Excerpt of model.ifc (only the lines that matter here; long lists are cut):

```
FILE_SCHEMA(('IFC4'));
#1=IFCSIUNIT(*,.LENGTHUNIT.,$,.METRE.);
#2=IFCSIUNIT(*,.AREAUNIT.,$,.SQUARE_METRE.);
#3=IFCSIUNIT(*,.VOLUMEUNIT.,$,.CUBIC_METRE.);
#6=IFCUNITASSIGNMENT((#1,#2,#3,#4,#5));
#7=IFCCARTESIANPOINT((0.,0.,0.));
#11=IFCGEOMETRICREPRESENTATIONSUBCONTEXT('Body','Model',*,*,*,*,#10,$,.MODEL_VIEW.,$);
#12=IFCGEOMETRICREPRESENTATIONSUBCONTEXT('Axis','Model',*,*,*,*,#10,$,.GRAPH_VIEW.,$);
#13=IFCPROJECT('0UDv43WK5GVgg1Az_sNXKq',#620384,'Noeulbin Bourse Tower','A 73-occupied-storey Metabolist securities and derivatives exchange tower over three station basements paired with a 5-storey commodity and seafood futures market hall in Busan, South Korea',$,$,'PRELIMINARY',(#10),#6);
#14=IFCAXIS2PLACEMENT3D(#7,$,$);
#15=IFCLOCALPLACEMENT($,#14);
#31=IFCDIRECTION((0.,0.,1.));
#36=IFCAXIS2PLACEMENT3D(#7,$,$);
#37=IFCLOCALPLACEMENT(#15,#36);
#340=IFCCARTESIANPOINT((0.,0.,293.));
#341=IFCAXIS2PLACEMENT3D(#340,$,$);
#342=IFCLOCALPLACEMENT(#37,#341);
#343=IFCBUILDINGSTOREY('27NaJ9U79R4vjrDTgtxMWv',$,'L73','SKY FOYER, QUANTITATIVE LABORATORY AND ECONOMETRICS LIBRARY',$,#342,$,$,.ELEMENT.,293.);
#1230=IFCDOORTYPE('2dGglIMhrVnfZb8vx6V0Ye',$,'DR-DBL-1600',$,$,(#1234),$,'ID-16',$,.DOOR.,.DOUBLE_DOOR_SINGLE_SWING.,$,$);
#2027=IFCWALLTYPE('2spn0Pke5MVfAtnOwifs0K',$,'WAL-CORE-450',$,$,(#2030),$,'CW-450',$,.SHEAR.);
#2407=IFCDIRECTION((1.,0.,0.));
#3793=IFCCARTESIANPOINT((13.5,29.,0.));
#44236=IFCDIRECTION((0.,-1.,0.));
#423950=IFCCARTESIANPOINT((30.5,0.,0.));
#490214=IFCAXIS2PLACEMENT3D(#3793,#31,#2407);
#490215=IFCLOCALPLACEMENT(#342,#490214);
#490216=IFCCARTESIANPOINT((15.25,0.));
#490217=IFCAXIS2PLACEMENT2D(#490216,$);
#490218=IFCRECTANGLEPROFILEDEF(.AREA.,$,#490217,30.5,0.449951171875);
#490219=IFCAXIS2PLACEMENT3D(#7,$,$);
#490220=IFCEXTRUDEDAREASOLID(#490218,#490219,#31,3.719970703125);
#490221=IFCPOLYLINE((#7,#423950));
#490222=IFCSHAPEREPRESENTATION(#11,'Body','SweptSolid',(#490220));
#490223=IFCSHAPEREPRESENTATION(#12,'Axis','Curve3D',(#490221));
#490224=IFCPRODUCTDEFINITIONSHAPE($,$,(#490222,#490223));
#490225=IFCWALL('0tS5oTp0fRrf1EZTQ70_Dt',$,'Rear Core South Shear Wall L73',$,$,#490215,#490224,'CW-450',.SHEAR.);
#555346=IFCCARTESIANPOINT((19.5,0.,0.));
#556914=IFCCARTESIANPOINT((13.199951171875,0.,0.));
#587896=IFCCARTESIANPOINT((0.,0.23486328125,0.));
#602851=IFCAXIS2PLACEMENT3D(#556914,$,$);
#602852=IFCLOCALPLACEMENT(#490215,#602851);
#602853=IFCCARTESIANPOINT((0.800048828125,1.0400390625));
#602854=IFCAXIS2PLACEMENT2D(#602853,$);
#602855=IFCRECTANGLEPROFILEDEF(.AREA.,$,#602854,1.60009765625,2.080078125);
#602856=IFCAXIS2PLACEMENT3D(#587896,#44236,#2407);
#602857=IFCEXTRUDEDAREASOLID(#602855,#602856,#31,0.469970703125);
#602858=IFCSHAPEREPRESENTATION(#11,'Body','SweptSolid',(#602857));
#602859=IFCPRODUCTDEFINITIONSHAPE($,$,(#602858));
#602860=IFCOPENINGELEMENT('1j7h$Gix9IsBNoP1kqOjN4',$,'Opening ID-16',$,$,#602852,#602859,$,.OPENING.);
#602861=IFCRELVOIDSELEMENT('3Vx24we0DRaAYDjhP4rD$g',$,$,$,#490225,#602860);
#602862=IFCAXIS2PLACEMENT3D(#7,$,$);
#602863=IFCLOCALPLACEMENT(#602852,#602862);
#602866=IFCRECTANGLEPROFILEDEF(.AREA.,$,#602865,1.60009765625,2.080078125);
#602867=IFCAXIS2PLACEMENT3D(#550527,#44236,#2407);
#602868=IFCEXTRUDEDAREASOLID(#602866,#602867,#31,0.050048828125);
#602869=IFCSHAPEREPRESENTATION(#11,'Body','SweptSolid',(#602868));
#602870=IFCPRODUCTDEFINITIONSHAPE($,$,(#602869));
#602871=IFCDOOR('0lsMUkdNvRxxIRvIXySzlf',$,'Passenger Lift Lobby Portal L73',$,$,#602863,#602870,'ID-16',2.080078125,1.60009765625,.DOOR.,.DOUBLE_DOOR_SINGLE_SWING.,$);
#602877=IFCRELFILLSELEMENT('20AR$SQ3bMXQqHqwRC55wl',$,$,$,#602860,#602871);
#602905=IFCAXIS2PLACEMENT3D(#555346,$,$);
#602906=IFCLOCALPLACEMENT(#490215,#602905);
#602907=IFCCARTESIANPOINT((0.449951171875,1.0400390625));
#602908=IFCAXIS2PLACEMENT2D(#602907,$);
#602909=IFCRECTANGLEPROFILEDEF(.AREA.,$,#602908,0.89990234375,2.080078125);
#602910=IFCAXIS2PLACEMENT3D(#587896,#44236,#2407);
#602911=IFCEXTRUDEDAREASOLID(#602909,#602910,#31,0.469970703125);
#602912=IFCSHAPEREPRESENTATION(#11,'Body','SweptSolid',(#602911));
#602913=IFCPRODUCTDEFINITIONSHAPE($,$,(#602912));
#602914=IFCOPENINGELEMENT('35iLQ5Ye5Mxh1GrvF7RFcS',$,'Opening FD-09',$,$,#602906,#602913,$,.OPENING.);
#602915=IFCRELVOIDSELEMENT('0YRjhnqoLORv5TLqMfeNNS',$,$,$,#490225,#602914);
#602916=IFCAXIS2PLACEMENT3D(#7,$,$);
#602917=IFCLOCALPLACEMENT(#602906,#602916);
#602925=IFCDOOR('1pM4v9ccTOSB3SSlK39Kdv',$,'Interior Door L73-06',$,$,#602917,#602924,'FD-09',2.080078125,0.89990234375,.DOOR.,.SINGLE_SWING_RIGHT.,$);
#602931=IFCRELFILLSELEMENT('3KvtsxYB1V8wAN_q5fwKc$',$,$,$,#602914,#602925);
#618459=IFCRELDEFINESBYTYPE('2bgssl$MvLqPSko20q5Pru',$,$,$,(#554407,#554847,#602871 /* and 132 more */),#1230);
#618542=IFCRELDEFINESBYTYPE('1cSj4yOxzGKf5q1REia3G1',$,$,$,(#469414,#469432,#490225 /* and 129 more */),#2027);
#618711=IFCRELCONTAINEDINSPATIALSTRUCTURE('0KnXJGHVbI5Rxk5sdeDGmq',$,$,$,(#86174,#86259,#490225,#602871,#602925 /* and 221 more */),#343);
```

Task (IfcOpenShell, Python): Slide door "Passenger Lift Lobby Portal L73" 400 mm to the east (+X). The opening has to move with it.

```python
import ifcopenshell
import ifcopenshell.api.geometry
import ifcopenshell.util.placement

model = ifcopenshell.open("model.ifc")

door = model.by_guid("0lsMUkdNvRxxIRvIXySzlf")
opening = door.FillsVoids[0].RelatingOpeningElement
wall = opening.VoidsElements[0].RelatingBuildingElement

wall_matrix = ifcopenshell.util.placement.get_local_placement(wall.ObjectPlacement)
shift = wall_matrix[:3, 0] * 0.4
before = ifcopenshell.util.placement.get_local_placement(door.ObjectPlacement)[:3, 3].copy()

# The door is placed relative to its opening, so it follows when the opening moves.
matrix = ifcopenshell.util.placement.get_local_placement(opening.ObjectPlacement)
matrix[:3, 3] += shift
ifcopenshell.api.geometry.edit_object_placement(
    model, product=opening, matrix=matrix, is_si=False, should_transform_children=True
)

after = ifcopenshell.util.placement.get_local_placement(door.ObjectPlacement)[:3, 3]
print("door moved by", (after - before).round(3) + 0.0)

model.write("model_updated.ifc")
```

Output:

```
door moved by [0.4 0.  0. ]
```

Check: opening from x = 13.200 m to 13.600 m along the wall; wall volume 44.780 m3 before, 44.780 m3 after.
